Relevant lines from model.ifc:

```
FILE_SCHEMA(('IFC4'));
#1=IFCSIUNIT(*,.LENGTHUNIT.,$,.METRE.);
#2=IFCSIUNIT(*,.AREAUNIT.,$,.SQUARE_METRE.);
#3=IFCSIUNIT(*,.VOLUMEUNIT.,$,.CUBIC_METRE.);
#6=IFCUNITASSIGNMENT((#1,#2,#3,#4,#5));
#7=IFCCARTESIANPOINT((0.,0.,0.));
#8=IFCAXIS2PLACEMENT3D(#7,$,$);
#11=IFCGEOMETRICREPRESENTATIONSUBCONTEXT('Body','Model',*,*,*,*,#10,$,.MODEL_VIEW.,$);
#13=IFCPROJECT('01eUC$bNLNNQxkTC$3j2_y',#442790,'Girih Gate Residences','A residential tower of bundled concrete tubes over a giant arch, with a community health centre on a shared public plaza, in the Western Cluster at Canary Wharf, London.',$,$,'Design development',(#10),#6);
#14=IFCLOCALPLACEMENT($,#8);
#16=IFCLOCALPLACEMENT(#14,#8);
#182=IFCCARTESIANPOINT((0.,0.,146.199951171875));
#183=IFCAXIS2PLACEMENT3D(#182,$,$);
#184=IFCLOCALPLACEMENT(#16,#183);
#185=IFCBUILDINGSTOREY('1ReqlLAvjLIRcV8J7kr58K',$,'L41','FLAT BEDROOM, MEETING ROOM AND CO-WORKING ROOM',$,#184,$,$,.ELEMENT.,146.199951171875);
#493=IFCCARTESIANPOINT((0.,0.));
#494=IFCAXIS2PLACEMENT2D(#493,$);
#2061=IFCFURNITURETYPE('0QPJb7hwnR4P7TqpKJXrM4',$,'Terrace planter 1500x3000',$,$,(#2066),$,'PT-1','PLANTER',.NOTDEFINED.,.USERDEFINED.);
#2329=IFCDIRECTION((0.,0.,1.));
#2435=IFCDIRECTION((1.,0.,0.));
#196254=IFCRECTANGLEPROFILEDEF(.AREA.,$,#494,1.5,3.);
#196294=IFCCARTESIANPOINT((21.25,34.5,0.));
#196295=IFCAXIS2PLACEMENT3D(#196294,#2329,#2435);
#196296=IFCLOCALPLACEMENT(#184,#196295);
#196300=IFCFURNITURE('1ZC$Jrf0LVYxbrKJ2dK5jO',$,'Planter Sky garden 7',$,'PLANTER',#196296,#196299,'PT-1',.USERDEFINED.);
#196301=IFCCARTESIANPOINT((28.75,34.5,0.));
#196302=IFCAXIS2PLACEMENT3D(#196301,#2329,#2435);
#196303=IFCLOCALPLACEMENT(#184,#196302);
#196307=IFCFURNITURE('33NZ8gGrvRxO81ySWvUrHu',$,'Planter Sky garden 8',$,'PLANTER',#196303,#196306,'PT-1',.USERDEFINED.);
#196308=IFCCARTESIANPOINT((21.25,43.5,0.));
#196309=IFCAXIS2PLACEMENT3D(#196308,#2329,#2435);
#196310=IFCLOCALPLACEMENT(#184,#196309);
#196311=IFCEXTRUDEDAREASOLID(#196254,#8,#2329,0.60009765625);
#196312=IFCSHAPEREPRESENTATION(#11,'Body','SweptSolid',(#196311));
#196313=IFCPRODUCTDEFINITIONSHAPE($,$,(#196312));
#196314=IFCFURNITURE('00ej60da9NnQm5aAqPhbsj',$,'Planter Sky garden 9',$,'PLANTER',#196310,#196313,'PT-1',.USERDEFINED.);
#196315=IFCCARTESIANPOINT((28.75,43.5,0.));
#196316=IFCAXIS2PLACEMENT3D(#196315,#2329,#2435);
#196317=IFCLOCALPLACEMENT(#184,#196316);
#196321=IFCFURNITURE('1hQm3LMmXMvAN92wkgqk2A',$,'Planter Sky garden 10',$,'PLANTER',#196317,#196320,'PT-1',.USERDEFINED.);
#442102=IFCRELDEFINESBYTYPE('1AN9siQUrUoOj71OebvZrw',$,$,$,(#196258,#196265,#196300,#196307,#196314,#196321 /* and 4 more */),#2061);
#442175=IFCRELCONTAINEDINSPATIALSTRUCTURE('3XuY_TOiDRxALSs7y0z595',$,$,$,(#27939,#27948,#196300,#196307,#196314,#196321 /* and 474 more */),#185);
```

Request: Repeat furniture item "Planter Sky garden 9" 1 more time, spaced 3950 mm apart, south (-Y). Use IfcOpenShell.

```python
import numpy as np
import ifcopenshell
import ifcopenshell.api.geometry
import ifcopenshell.api.root
import ifcopenshell.util.element
import ifcopenshell.util.placement
import ifcopenshell.util.unit

model = ifcopenshell.open("model.ifc")
unit_scale = ifcopenshell.util.unit.calculate_unit_scale(model)

source = model.by_guid("00ej60da9NnQm5aAqPhbsj")
base = ifcopenshell.util.placement.get_local_placement(source.ObjectPlacement)
step = np.array([0.0, -1.0, 0.0]) * 3.95 / unit_scale

for i in range(1, 2):
    copy = ifcopenshell.api.root.copy_class(model, product=source)
    copy.Representation = ifcopenshell.util.element.copy_deep(
        model, source.Representation, exclude=["IfcGeometricRepresentationContext", "IfcRepresentationMap"]
    )
    copy.Tag = None
    matrix = base.copy()
    matrix[:3, 3] += i * step
    print("added at", matrix[:3, 3].round(3) + 0.0)
    ifcopenshell.api.geometry.edit_object_placement(model, product=copy, matrix=matrix, is_si=False)

model.write("model-out.ifc")
```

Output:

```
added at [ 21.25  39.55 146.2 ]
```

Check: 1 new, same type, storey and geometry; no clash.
